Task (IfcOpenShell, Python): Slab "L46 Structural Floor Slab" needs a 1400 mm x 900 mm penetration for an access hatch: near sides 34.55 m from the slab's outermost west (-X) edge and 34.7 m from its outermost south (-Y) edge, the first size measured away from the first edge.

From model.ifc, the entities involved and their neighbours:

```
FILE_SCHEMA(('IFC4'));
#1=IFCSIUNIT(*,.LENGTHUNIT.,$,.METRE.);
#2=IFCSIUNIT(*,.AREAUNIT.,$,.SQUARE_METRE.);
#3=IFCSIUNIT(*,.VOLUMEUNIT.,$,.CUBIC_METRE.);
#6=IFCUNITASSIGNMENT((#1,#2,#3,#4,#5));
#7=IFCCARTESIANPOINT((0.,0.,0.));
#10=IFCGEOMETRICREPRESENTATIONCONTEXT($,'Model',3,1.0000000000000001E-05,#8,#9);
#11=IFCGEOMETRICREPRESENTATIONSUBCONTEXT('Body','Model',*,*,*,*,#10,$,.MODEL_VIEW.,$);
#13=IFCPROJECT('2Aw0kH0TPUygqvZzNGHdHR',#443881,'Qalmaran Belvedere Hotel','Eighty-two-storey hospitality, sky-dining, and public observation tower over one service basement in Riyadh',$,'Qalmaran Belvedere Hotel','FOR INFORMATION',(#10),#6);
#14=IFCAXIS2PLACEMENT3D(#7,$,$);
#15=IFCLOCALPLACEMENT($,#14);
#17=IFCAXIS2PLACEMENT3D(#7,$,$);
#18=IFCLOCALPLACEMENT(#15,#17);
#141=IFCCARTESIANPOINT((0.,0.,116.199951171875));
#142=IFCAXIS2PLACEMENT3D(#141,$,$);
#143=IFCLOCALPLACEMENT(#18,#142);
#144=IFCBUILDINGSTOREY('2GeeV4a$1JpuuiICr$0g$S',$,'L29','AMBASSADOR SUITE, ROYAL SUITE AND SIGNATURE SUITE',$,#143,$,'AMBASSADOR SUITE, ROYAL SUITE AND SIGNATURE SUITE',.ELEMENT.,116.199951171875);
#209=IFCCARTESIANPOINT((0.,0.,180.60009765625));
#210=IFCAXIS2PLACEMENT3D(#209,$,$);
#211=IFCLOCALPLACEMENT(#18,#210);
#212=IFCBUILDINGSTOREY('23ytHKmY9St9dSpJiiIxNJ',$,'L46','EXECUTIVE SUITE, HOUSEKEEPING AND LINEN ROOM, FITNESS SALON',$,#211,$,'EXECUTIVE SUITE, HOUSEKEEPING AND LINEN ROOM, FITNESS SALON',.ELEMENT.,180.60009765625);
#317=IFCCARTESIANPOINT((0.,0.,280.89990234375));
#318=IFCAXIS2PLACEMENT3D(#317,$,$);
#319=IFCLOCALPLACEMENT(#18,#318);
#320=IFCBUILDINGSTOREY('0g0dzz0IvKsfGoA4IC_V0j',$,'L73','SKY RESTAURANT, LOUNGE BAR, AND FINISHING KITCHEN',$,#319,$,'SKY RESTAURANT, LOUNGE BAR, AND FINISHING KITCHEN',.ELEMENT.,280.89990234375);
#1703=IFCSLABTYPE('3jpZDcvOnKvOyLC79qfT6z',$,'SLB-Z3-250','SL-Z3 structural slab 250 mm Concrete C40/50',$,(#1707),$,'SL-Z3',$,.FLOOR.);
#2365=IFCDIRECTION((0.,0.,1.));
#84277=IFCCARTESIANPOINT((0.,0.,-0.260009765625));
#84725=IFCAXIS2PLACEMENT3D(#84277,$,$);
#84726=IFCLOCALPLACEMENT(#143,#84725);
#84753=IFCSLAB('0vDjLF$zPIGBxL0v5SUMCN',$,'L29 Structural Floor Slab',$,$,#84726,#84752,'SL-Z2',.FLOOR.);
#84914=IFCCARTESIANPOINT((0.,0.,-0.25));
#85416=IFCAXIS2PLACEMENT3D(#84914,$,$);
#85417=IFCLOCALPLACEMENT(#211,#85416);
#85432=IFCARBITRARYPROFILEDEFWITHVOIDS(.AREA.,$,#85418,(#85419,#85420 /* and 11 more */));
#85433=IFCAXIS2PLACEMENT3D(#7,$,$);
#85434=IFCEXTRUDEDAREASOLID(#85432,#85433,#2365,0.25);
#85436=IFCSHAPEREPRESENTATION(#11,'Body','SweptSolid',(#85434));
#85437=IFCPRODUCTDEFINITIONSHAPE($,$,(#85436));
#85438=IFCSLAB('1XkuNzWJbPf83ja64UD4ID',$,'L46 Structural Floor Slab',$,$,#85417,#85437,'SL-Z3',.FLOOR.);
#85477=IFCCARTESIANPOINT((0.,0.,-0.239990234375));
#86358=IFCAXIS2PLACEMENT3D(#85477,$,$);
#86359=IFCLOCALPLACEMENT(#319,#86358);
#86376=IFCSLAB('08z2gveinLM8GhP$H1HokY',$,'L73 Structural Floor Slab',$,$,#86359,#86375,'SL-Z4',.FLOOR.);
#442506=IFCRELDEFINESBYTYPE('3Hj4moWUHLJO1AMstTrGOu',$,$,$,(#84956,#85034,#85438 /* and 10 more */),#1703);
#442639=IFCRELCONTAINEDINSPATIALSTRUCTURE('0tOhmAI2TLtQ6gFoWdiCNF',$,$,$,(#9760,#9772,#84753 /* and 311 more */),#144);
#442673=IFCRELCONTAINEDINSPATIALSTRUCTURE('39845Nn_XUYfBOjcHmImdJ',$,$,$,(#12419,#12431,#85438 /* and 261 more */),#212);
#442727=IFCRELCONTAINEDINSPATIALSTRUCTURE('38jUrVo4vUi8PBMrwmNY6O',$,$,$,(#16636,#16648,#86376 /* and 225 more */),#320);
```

```python
import numpy as np
import ifcopenshell
import ifcopenshell.api.feature
import ifcopenshell.api.geometry
import ifcopenshell.api.root
import ifcopenshell.geom
import ifcopenshell.util.placement
import ifcopenshell.util.representation
import ifcopenshell.util.shape
import ifcopenshell.util.unit

model = ifcopenshell.open("model.ifc")
unit_scale = ifcopenshell.util.unit.calculate_unit_scale(model)
settings = ifcopenshell.geom.settings()


def volume(element):
    """Net volume in cubic metres, openings subtracted."""
    shape = ifcopenshell.geom.create_shape(settings, element)
    return ifcopenshell.util.shape.get_volume(shape.geometry)


slab = model.by_id(85438)
before = volume(slab)

# Extent in the slab's own axes, in metres. The edges named are its -X and -Y sides.
slab_shape = ifcopenshell.geom.create_shape(settings, slab)
vertices = ifcopenshell.util.shape.get_vertices(slab_shape.geometry)
x_min, y_min, bottom = vertices.min(axis=0)
top = vertices[:, 2].max()

opening = ifcopenshell.api.root.create_entity(model, ifc_class="IfcOpeningElement", name="Access hatch opening", predefined_type="OPENING")
context = ifcopenshell.util.representation.get_context(model, "Model", "Body", "MODEL_VIEW")
width, depth = 1.4, 0.9
outline = [(0.0, 0.0), (width, 0.0), (width, depth), (0.0, depth), (0.0, 0.0)]
# Overshoot both faces by 50 mm so the cut is clean.
shape = ifcopenshell.api.geometry.add_slab_representation(
    model, context=context, depth=top - bottom + 0.1, polyline=outline
)
ifcopenshell.api.geometry.assign_representation(model, product=opening, representation=shape)

matrix = ifcopenshell.util.placement.get_local_placement(slab.ObjectPlacement)
matrix[:, 3] = matrix @ np.append(np.array([x_min + 34.55, y_min + 34.7, bottom - 0.05]) / unit_scale, 1.0)
ifcopenshell.api.geometry.edit_object_placement(model, product=opening, matrix=matrix, is_si=False)
ifcopenshell.api.feature.add_feature(model, feature=opening, element=slab)

after = volume(slab)

print(f"slab volume {before:.3f} -> {after:.3f} m3")

model.write("model_rev.ifc")
```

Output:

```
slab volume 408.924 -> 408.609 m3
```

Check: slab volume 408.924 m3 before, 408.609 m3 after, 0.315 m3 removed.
